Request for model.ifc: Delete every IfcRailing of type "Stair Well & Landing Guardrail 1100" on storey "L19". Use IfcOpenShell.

First a look at what the model holds.

```python
import ifcopenshell
import ifcopenshell.util.element

model = ifcopenshell.open("model.ifc")
print(model.schema)
storey = next(s for s in model.by_type("IfcBuildingStorey") if s.Name == "L19")
railings = [e for e in ifcopenshell.util.element.get_decomposition(storey) if e.is_a("IfcRailing")]
seen = {}
for e in railings:
    element_type = ifcopenshell.util.element.get_type(e)
    name = element_type.Name if element_type not in (None, e) else None
    seen[name] = seen.get(name, 0) + 1
for name, count in sorted(seen.items(), key=str):
    print(count, "x", name)
```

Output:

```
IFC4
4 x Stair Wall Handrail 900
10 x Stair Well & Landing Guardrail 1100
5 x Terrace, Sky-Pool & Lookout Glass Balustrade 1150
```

```python
import ifcopenshell
import ifcopenshell.api.root
import ifcopenshell.util.element

model = ifcopenshell.open("model.ifc")

storey = next(s for s in model.by_type("IfcBuildingStorey") if s.Name == "L19")
railings = [e for e in ifcopenshell.util.element.get_decomposition(storey) if e.is_a("IfcRailing")]
targets = [e for e in railings if (t := ifcopenshell.util.element.get_type(e)) not in (None, e) and t.Name == "Stair Well & Landing Guardrail 1100"]

for e in targets:
    ifcopenshell.api.root.remove_product(model, product=e)
print(len(targets), "removed")

model.write("model_rev.ifc")
```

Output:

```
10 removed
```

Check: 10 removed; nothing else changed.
